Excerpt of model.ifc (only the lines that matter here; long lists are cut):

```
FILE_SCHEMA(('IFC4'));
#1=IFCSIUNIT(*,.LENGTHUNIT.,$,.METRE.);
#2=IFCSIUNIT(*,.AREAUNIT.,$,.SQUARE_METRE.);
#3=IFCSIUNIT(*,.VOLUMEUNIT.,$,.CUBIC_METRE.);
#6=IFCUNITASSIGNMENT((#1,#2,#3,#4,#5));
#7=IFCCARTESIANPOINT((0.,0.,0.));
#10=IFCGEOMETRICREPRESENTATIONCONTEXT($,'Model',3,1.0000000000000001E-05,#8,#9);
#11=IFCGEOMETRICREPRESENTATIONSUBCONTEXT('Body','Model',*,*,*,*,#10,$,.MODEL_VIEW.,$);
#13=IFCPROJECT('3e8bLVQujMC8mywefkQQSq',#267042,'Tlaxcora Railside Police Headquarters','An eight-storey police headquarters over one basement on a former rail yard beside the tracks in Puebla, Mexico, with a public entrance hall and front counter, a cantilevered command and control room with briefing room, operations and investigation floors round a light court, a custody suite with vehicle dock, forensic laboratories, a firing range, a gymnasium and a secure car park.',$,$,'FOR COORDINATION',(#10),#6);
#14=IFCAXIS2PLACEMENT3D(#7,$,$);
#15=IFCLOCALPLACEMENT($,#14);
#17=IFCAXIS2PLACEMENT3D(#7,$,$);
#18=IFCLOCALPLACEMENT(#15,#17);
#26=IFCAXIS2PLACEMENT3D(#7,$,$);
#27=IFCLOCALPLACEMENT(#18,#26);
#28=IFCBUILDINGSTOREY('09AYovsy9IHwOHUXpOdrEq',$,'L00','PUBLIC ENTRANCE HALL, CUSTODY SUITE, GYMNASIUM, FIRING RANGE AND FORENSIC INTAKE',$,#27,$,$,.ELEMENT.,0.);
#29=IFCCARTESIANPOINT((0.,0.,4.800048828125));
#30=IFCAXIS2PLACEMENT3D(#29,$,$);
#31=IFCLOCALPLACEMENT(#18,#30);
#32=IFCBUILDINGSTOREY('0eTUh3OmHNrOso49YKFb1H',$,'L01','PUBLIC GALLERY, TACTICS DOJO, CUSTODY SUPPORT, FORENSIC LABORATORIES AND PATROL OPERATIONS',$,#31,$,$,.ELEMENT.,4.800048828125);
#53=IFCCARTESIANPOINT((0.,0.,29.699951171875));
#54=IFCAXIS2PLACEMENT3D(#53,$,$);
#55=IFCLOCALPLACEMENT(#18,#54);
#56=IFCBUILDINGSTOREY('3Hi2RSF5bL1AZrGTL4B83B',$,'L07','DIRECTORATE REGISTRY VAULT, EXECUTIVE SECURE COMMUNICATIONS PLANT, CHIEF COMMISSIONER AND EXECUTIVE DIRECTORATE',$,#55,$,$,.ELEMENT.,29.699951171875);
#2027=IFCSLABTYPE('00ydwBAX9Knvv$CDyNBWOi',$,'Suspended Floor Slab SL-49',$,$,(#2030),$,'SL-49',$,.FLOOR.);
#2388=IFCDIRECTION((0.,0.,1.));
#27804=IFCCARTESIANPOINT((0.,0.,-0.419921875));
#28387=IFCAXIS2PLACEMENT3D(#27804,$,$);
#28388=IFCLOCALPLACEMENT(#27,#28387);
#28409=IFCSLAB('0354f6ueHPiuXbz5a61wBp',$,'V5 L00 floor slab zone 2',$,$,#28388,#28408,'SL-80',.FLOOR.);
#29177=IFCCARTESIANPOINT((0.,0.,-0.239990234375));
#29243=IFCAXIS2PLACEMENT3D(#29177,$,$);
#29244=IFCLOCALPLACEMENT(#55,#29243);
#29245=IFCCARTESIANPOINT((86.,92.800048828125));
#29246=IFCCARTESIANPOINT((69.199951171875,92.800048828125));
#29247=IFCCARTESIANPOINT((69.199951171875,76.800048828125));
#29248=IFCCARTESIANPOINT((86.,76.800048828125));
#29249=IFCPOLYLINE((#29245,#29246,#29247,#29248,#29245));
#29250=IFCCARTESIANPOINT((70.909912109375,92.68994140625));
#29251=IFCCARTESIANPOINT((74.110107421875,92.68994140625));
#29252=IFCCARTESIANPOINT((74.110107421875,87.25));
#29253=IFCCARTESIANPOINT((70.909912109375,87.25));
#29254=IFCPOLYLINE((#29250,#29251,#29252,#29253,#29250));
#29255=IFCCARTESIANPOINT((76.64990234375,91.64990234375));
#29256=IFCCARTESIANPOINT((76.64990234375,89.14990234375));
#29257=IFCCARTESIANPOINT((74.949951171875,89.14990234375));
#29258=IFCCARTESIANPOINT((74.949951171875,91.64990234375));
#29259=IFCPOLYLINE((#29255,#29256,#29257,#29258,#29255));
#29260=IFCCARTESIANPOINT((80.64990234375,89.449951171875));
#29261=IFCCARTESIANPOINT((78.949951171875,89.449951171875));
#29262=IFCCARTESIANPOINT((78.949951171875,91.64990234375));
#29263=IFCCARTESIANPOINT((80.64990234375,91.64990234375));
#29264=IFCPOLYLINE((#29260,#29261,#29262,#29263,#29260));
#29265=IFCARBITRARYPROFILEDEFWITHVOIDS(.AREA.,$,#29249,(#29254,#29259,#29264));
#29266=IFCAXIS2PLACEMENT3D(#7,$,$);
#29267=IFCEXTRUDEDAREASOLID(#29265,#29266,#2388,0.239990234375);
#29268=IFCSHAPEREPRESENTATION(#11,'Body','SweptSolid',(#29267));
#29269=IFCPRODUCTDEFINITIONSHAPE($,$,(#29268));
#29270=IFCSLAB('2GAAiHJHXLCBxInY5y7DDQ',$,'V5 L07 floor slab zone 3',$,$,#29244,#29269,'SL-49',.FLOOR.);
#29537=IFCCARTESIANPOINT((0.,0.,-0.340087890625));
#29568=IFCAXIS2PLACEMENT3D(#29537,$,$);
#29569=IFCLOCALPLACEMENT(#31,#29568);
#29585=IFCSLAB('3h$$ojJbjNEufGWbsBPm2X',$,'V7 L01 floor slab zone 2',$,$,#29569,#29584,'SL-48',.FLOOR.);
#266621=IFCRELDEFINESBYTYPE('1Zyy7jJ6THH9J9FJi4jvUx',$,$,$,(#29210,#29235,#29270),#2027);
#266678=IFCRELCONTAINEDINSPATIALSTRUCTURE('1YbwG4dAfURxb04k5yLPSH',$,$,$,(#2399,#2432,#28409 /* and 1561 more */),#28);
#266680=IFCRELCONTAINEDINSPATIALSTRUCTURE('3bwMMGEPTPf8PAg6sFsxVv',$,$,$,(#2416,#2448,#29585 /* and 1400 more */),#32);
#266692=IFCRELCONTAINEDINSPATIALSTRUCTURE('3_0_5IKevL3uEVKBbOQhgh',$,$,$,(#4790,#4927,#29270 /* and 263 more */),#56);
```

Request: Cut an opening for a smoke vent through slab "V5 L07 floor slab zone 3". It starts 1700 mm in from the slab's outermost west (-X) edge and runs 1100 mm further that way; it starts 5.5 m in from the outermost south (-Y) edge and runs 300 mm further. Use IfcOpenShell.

```python
import numpy as np
import ifcopenshell
import ifcopenshell.api.feature
import ifcopenshell.api.geometry
import ifcopenshell.api.root
import ifcopenshell.geom
import ifcopenshell.util.placement
import ifcopenshell.util.representation
import ifcopenshell.util.shape
import ifcopenshell.util.unit

model = ifcopenshell.open("model.ifc")
unit_scale = ifcopenshell.util.unit.calculate_unit_scale(model)
settings = ifcopenshell.geom.settings()


def volume(element):
    """Net volume in cubic metres, openings subtracted."""
    shape = ifcopenshell.geom.create_shape(settings, element)
    return ifcopenshell.util.shape.get_volume(shape.geometry)


slab = model.by_guid("2GAAiHJHXLCBxInY5y7DDQ")
before = volume(slab)

# Extent in the slab's own axes, in metres. The edges named are its -X and -Y sides.
slab_shape = ifcopenshell.geom.create_shape(settings, slab)
vertices = ifcopenshell.util.shape.get_vertices(slab_shape.geometry)
x_min, y_min, bottom = vertices.min(axis=0)
top = vertices[:, 2].max()

opening = ifcopenshell.api.root.create_entity(model, ifc_class="IfcOpeningElement", name="Smoke vent opening", predefined_type="OPENING")
context = ifcopenshell.util.representation.get_context(model, "Model", "Body", "MODEL_VIEW")
width, depth = 1.1, 0.3
outline = [(0.0, 0.0), (width, 0.0), (width, depth), (0.0, depth), (0.0, 0.0)]
# Overshoot both faces by 50 mm so the cut is clean.
shape = ifcopenshell.api.geometry.add_slab_representation(
    model, context=context, depth=top - bottom + 0.1, polyline=outline
)
ifcopenshell.api.geometry.assign_representation(model, product=opening, representation=shape)

matrix = ifcopenshell.util.placement.get_local_placement(slab.ObjectPlacement)
matrix[:, 3] = matrix @ np.append(np.array([x_min + 1.7, y_min + 5.5, bottom - 0.05]) / unit_scale, 1.0)
ifcopenshell.api.geometry.edit_object_placement(model, product=opening, matrix=matrix, is_si=False)
ifcopenshell.api.feature.add_feature(model, feature=opening, element=slab)

after = volume(slab)

print(f"slab volume {before:.3f} -> {after:.3f} m3")

model.write("model_rev.ifc")
```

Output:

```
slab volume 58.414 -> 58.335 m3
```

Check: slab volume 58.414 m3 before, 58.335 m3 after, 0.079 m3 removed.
